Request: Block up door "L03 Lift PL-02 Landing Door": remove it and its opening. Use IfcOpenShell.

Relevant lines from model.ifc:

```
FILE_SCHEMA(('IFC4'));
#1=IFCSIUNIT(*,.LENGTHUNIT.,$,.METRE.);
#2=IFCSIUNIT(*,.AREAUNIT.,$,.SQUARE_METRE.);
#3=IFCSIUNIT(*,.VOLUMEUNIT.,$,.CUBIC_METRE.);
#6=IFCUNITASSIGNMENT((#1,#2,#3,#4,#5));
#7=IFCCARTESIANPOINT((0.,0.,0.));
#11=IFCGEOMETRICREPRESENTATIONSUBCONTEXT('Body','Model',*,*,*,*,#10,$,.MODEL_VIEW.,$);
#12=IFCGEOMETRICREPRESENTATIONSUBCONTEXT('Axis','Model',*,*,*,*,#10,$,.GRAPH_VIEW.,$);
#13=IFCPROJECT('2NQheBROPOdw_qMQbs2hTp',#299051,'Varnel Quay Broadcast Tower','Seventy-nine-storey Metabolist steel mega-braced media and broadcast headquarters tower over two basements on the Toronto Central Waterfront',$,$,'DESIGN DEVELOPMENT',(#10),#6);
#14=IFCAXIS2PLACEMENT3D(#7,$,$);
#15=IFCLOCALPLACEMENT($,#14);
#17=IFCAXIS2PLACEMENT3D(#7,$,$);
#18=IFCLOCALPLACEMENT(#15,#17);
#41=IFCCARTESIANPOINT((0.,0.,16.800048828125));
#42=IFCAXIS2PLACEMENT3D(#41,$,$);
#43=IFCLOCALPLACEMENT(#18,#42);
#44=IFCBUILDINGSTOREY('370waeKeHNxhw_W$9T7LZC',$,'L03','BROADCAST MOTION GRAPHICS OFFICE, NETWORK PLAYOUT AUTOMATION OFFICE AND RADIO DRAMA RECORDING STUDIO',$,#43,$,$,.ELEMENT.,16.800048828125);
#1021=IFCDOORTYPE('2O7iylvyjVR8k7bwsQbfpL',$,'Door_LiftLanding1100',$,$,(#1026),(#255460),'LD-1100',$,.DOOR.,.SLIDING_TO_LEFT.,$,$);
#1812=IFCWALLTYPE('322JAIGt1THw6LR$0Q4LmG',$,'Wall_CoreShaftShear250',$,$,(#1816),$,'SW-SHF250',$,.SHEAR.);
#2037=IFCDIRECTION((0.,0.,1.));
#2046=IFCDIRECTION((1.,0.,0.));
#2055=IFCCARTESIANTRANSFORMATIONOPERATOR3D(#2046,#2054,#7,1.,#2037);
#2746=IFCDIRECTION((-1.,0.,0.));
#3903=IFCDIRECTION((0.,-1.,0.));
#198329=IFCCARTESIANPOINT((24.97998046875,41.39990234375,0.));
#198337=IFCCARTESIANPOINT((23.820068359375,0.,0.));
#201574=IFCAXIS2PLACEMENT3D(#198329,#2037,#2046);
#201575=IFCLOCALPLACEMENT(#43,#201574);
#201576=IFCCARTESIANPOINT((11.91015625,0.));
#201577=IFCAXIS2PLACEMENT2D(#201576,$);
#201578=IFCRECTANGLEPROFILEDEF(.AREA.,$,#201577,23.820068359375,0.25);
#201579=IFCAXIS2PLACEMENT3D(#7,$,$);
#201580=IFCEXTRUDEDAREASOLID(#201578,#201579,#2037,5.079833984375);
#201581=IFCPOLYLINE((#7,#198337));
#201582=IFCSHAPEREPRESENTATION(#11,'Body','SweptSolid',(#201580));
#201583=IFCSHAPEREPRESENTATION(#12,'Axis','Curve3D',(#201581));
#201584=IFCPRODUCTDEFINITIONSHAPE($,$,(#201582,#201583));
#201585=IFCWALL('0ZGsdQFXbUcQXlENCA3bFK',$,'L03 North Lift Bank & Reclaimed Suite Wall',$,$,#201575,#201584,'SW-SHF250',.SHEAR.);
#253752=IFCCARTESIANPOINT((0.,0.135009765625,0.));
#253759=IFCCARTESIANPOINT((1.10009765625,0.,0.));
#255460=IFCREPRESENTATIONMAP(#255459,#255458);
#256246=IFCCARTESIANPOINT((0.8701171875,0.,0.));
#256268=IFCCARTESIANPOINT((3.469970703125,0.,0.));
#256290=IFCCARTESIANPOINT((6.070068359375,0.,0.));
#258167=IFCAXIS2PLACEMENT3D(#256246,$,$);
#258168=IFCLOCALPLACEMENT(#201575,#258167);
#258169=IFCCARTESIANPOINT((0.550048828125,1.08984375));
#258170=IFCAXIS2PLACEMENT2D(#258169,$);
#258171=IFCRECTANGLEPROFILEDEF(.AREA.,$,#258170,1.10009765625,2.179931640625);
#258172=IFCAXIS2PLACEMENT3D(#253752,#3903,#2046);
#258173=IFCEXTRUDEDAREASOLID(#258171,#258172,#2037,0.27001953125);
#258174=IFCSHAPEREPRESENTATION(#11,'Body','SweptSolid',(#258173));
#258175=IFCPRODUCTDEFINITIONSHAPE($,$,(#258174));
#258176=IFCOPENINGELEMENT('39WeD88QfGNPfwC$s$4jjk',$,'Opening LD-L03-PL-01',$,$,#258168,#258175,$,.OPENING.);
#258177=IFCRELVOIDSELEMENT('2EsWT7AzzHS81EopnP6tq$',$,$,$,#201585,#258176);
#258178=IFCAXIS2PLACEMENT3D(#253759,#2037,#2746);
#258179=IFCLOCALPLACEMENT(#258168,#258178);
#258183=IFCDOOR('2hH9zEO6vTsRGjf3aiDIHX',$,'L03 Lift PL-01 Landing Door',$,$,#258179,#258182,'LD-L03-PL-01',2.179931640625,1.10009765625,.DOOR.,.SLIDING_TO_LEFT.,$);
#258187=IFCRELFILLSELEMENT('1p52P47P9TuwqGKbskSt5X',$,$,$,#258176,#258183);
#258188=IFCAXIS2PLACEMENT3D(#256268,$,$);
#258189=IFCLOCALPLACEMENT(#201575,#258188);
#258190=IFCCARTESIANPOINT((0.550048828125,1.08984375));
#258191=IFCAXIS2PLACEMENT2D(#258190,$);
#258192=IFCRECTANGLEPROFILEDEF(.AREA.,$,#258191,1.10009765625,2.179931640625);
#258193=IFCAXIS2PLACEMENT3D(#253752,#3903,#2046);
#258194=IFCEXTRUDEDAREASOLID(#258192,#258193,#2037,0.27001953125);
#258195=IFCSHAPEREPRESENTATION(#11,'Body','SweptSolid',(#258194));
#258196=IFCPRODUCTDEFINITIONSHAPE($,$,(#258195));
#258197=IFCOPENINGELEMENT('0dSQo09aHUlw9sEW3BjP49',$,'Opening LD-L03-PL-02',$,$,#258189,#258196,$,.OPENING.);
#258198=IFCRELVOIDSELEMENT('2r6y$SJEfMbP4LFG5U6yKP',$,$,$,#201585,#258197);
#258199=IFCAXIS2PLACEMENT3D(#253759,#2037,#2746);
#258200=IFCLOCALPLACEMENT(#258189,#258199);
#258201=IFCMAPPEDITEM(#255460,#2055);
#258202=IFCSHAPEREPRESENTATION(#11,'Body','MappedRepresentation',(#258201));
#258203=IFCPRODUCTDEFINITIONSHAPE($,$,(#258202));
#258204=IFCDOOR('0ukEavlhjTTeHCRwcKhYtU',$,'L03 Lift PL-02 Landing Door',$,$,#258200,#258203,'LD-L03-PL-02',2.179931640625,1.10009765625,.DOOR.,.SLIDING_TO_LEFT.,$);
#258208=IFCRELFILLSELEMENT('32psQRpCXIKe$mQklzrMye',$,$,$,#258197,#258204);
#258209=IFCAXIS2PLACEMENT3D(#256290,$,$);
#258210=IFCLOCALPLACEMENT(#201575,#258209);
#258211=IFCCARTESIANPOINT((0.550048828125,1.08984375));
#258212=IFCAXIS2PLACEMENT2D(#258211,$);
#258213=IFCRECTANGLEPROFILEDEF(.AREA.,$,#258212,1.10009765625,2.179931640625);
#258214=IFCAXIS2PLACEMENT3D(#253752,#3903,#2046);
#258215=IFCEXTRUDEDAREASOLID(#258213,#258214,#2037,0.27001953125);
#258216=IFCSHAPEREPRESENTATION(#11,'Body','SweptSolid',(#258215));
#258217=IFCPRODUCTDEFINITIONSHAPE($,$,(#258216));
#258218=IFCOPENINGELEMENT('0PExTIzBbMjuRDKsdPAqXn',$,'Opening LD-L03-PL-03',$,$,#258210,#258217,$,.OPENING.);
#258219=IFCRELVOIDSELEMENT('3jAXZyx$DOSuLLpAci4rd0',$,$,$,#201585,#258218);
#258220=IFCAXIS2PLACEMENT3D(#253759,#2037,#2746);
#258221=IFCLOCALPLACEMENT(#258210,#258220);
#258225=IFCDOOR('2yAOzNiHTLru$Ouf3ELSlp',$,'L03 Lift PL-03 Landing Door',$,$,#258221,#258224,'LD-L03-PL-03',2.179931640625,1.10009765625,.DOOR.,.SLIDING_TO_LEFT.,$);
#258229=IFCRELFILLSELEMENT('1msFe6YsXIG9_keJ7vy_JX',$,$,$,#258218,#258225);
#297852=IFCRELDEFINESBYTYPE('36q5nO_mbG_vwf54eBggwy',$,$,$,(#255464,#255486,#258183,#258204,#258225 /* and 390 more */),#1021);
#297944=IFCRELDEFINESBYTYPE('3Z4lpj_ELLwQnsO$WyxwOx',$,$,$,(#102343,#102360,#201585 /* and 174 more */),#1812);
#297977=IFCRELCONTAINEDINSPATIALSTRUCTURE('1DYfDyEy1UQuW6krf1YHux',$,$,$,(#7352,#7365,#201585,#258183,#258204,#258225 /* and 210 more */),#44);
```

```python
import ifcopenshell
import ifcopenshell.api.feature
import ifcopenshell.api.root
import ifcopenshell.geom
import ifcopenshell.util.shape

model = ifcopenshell.open("model.ifc")
settings = ifcopenshell.geom.settings()


def volume(element):
    """Net volume in cubic metres, openings subtracted."""
    shape = ifcopenshell.geom.create_shape(settings, element)
    return ifcopenshell.util.shape.get_volume(shape.geometry)


door = model.by_guid("0ukEavlhjTTeHCRwcKhYtU")
opening = door.FillsVoids[0].RelatingOpeningElement
wall = opening.VoidsElements[0].RelatingBuildingElement
before = volume(wall)

ifcopenshell.api.root.remove_product(model, product=door)
ifcopenshell.api.feature.remove_feature(model, feature=opening)

after = volume(wall)

print(f"wall volume {before:.3f} -> {after:.3f} m3")

model.write("model_rev.ifc")
```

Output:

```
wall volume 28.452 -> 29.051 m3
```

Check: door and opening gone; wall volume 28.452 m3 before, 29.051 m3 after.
